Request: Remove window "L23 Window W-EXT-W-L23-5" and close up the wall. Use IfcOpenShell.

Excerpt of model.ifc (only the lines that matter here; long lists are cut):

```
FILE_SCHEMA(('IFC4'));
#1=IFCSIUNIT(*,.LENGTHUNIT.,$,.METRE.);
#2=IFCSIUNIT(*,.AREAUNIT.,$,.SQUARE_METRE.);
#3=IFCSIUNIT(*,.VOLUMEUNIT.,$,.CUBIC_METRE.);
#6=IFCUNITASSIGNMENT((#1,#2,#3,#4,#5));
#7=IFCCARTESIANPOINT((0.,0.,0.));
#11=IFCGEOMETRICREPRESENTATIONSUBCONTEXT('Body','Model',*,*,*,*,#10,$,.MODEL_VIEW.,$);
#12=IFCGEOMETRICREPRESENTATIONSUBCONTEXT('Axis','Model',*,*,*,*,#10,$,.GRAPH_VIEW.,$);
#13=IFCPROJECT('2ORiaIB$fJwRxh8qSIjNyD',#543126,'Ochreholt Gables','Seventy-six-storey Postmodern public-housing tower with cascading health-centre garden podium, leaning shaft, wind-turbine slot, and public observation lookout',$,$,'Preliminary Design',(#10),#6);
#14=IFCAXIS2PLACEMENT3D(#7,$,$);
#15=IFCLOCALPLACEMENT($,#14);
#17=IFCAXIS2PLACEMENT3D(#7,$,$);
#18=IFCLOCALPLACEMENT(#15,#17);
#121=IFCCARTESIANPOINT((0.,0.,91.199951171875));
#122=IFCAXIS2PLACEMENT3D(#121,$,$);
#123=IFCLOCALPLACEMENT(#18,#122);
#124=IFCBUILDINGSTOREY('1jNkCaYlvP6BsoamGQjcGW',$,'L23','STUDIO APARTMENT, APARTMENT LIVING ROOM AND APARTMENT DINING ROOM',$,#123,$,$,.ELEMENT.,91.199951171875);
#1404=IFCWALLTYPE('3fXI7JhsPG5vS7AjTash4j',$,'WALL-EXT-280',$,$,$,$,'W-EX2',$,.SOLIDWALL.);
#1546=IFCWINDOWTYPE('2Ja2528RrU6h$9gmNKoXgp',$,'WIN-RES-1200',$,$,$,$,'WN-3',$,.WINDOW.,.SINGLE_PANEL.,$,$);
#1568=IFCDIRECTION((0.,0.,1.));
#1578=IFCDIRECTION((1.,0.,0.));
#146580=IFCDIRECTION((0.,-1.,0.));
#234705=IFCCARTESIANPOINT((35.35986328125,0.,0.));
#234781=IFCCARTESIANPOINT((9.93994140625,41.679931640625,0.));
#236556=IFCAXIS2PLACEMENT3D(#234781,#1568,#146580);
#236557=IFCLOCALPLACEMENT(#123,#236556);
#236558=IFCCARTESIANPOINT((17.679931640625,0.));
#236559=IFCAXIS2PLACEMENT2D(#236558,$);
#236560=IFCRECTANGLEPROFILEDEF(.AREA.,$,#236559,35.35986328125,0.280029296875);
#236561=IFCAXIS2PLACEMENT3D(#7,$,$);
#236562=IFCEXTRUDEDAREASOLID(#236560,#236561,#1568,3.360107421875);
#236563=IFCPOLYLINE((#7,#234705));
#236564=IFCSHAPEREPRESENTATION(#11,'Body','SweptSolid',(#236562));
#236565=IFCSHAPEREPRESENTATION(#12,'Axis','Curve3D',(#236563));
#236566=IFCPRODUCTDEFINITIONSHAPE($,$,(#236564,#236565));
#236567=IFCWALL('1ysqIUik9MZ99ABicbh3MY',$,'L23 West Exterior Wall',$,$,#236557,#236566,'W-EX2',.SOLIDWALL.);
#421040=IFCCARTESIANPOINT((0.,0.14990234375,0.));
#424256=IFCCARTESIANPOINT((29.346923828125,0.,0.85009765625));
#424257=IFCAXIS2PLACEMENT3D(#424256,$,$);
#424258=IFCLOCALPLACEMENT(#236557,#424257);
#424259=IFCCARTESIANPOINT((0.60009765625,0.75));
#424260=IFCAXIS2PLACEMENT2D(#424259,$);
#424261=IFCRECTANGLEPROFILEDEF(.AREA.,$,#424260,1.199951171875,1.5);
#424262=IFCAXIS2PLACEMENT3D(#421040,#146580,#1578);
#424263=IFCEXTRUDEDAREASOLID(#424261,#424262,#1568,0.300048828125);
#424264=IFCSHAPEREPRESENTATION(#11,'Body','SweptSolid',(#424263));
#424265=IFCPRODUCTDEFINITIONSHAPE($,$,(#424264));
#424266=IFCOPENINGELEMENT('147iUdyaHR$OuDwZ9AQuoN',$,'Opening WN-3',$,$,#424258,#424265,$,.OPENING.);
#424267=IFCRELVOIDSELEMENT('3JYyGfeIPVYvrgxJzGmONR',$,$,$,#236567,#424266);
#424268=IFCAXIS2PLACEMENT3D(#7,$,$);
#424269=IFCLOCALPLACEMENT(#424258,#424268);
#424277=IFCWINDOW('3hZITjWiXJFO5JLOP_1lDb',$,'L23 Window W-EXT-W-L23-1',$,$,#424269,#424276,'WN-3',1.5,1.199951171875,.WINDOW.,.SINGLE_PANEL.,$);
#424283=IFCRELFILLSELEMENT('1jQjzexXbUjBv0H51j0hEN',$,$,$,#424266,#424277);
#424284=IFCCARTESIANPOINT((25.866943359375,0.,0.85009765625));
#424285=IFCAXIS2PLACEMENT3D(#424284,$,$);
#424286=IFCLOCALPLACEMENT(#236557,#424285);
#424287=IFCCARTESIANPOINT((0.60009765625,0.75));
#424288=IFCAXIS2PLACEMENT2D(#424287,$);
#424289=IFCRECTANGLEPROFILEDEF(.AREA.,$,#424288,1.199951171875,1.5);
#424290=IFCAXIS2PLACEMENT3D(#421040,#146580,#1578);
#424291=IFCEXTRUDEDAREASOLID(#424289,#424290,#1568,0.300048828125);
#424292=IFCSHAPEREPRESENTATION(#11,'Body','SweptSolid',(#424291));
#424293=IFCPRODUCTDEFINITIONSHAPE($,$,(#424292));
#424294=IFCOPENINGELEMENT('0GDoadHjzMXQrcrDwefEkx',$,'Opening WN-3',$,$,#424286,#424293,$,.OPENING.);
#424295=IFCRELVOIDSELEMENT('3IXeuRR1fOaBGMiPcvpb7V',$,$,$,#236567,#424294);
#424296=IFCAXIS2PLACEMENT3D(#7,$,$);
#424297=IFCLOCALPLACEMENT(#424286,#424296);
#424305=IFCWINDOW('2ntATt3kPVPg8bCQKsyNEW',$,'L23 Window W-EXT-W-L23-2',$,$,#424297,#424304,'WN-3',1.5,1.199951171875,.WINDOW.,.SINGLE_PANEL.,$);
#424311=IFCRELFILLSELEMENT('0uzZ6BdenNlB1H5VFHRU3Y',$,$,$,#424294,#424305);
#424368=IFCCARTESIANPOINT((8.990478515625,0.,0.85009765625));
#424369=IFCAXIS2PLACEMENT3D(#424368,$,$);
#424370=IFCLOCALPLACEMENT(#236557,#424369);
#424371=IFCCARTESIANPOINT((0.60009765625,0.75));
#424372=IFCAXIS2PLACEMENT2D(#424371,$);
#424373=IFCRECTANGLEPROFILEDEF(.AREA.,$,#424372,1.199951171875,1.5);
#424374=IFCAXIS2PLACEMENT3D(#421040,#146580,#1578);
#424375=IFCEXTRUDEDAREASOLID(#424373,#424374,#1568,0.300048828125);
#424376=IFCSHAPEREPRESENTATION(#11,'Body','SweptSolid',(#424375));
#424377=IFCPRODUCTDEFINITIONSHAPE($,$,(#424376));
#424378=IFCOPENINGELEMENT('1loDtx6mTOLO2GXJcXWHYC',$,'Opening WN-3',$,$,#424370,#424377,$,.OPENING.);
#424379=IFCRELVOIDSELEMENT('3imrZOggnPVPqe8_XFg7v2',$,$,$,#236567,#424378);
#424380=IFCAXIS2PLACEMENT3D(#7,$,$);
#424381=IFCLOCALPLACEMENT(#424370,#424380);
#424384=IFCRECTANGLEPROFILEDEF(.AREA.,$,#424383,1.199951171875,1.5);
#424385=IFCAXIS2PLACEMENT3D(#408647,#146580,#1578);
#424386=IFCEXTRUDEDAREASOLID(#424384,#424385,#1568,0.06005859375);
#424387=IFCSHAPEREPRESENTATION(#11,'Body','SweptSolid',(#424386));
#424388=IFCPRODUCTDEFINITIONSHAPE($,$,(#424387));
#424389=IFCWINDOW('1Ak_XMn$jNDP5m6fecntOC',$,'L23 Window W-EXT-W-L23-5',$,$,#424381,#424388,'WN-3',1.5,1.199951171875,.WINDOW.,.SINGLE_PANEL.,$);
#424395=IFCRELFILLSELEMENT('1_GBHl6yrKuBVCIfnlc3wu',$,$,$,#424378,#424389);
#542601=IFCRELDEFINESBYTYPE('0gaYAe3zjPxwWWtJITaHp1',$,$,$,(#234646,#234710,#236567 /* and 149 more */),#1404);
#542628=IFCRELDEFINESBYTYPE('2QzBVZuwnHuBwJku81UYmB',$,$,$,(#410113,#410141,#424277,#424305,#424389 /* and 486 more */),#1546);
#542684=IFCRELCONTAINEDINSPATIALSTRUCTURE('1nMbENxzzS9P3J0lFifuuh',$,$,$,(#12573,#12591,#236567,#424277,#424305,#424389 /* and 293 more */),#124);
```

```python
import ifcopenshell
import ifcopenshell.api.feature
import ifcopenshell.api.root
import ifcopenshell.geom
import ifcopenshell.util.shape

model = ifcopenshell.open("model.ifc")
settings = ifcopenshell.geom.settings()


def volume(element):
    """Net volume in cubic metres, openings subtracted."""
    shape = ifcopenshell.geom.create_shape(settings, element)
    return ifcopenshell.util.shape.get_volume(shape.geometry)


window = model.by_id(424389)
opening = window.FillsVoids[0].RelatingOpeningElement
wall = opening.VoidsElements[0].RelatingBuildingElement
before = volume(wall)

ifcopenshell.api.root.remove_product(model, product=window)
ifcopenshell.api.feature.remove_feature(model, feature=opening)

after = volume(wall)

print(f"wall volume {before:.3f} -> {after:.3f} m3")

model.write("model_edited.ifc")
```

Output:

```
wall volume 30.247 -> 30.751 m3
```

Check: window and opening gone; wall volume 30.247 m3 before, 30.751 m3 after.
